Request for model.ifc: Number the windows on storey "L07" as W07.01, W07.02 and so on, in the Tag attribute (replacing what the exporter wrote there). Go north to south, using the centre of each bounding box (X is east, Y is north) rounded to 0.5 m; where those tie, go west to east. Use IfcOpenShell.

First a look at what the model holds.

```python
import ifcopenshell
import ifcopenshell.util.element
import ifcopenshell.util.placement

model = ifcopenshell.open("model.ifc")
print(model.schema)
storey = next(s for s in model.by_type("IfcBuildingStorey") if s.Name == "L07")
windows = [e for e in ifcopenshell.util.element.get_decomposition(storey) if e.is_a("IfcWindow")]
for e in sorted(windows, key=lambda e: e.id()):
    origin = ifcopenshell.util.placement.get_local_placement(e.ObjectPlacement)[:3, 3]
    print(e.id(), e.Tag, e.Name, origin.round(2) + 0.0, sep=" | ")
```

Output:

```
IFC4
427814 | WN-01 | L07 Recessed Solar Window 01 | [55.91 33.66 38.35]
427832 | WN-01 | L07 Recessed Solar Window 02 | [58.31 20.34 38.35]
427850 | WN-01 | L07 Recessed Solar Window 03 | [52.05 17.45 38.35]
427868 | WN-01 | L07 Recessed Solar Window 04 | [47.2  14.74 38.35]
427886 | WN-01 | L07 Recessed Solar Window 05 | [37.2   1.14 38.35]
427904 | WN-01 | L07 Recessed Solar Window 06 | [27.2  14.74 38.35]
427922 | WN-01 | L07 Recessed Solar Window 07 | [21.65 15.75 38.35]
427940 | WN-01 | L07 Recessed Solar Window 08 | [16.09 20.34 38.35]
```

```python
import ifcopenshell
import ifcopenshell.geom
import ifcopenshell.util.element
import ifcopenshell.util.shape

model = ifcopenshell.open("model.ifc")
settings = ifcopenshell.geom.settings()
settings.set("use-world-coords", True)


def centre(element):
    shape = ifcopenshell.geom.create_shape(settings, element)
    return ifcopenshell.util.shape.get_bbox_centroid(shape.geometry)


storey = next(s for s in model.by_type("IfcBuildingStorey") if s.Name == "L07")
windows = [e for e in ifcopenshell.util.element.get_decomposition(storey) if e.is_a("IfcWindow")]

# Insertion points can sit at a corner or the storey origin, so sort by the geometry (in metres).
centres = {e: centre(e) for e in windows}
windows.sort(key=lambda e: (-round(centres[e][1] / 0.5), centres[e][0]))

for i, e in enumerate(windows, start=1):
    number = f"W07.{i:02d}"
    e.Tag = number
    print(e.id(), number)

model.write("model_edited.ifc")
```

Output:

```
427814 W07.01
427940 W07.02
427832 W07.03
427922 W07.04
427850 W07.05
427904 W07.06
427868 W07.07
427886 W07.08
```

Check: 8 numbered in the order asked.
